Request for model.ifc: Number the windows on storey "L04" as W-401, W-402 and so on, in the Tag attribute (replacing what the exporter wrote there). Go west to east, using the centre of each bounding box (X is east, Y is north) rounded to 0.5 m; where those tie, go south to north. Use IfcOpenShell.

First a look at what the model holds.

```python
import ifcopenshell
import ifcopenshell.util.element
import ifcopenshell.util.placement

model = ifcopenshell.open("model.ifc")
print(model.schema)
storey = next(s for s in model.by_type("IfcBuildingStorey") if s.Name == "L04")
windows = [e for e in ifcopenshell.util.element.get_decomposition(storey) if e.is_a("IfcWindow")]
for e in sorted(windows, key=lambda e: e.id()):
    origin = ifcopenshell.util.placement.get_local_placement(e.ObjectPlacement)[:3, 3]
    print(e.id(), e.Tag, e.Name, origin.round(2) + 0.0, sep=" | ")
```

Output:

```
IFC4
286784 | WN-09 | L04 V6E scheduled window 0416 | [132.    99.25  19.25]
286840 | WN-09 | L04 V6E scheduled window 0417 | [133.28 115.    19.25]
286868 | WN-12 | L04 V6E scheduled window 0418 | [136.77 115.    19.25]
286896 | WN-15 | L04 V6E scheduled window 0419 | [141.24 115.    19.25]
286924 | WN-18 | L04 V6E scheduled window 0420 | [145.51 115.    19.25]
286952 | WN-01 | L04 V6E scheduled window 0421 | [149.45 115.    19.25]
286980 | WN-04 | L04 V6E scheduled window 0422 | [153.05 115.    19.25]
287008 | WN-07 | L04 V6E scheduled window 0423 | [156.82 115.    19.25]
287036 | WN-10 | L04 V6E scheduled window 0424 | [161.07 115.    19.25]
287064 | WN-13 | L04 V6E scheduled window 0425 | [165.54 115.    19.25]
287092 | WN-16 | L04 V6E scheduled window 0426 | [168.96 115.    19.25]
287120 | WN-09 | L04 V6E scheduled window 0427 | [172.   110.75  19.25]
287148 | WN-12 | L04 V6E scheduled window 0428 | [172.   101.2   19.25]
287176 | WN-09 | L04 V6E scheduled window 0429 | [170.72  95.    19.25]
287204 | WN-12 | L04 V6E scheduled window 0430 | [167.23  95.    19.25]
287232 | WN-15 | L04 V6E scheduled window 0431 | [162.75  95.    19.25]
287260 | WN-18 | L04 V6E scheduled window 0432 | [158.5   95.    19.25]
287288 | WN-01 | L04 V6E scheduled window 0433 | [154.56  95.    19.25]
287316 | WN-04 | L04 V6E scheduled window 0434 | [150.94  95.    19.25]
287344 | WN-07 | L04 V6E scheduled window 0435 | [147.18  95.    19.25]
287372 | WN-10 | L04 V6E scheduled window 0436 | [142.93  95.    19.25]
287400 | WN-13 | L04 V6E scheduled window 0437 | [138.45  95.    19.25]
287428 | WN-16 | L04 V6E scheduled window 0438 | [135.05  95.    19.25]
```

```python
import ifcopenshell
import ifcopenshell.geom
import ifcopenshell.util.element
import ifcopenshell.util.shape

model = ifcopenshell.open("model.ifc")
settings = ifcopenshell.geom.settings()
settings.set("use-world-coords", True)


def centre(element):
    shape = ifcopenshell.geom.create_shape(settings, element)
    return ifcopenshell.util.shape.get_bbox_centroid(shape.geometry)


storey = next(s for s in model.by_type("IfcBuildingStorey") if s.Name == "L04")
windows = [e for e in ifcopenshell.util.element.get_decomposition(storey) if e.is_a("IfcWindow")]

# Insertion points can sit at a corner or the storey origin, so sort by the geometry (in metres).
centres = {e: centre(e) for e in windows}
windows.sort(key=lambda e: (round(centres[e][0] / 0.5), centres[e][1]))

for i, e in enumerate(windows, start=1):
    number = f"W-4{i:02d}"
    e.Tag = number
    print(e.id(), number)

model.write("model_edited.ifc")
```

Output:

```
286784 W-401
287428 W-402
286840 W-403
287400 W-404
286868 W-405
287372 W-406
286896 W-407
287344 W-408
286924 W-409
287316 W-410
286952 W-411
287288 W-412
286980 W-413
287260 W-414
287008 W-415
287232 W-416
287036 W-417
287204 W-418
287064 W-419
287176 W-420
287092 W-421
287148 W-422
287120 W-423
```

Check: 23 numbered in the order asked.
